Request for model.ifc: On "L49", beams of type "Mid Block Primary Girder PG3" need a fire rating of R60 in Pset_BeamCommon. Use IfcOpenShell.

First a look at what the model holds.

```python
import ifcopenshell
import ifcopenshell.util.element

model = ifcopenshell.open("model.ifc")
print(model.schema)
storey = next(s for s in model.by_type("IfcBuildingStorey") if s.Name == "L49")
beams = [e for e in ifcopenshell.util.element.get_decomposition(storey) if e.is_a("IfcBeam")]
seen = {}
for e in beams:
    element_type = ifcopenshell.util.element.get_type(e)
    key = (element_type.Name if element_type != e and element_type else None, ifcopenshell.util.element.get_pset(e, "Pset_BeamCommon", "FireRating"))
    seen[key] = seen.get(key, 0) + 1
for (name, value), count in sorted(seen.items(), key=str):
    print(count, "x", name, "|", value)
```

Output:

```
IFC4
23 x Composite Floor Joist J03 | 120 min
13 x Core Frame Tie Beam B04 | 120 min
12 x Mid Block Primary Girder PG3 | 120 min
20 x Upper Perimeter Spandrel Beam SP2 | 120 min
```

```python
import ifcopenshell
import ifcopenshell.api.pset
import ifcopenshell.util.element

model = ifcopenshell.open("model.ifc")

storey = next(s for s in model.by_type("IfcBuildingStorey") if s.Name == "L49")
beams = [e for e in ifcopenshell.util.element.get_decomposition(storey) if e.is_a("IfcBeam")]

count = 0
for e in beams:
    element_type = ifcopenshell.util.element.get_type(e)
    if element_type in (None, e) or element_type.Name != "Mid Block Primary Girder PG3":
        continue
    found = ifcopenshell.util.element.get_pset(e, "Pset_BeamCommon", should_inherit=False)
    if found:
        pset = model.by_id(found["id"])
        if len(ifcopenshell.util.element.get_elements_by_pset(pset)) > 1:
            pset = ifcopenshell.api.pset.unshare_pset(model, products=[e], pset=pset)[0]
    else:
        pset = ifcopenshell.api.pset.add_pset(model, product=e, name="Pset_BeamCommon")
    ifcopenshell.api.pset.edit_pset(model, pset=pset, properties={"FireRating": "R60"})
    count += 1

print(count, "beams updated")

model.write("model_edited.ifc")
```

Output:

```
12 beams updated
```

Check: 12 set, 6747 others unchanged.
